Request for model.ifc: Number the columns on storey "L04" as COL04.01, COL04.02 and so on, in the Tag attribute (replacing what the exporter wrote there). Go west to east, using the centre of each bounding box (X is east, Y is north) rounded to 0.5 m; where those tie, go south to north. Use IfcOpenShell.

First a look at what the model holds.

```python
import ifcopenshell
import ifcopenshell.util.element
import ifcopenshell.util.placement

model = ifcopenshell.open("model.ifc")
print(model.schema)
storey = next(s for s in model.by_type("IfcBuildingStorey") if s.Name == "L04")
columns = [e for e in ifcopenshell.util.element.get_decomposition(storey) if e.is_a("IfcColumn")]
for e in sorted(columns, key=lambda e: e.id()):
    origin = ifcopenshell.util.placement.get_local_placement(e.ObjectPlacement)[:3, 3]
    print(e.id(), e.Tag, e.Name, origin.round(2) + 0.0, sep=" | ")
```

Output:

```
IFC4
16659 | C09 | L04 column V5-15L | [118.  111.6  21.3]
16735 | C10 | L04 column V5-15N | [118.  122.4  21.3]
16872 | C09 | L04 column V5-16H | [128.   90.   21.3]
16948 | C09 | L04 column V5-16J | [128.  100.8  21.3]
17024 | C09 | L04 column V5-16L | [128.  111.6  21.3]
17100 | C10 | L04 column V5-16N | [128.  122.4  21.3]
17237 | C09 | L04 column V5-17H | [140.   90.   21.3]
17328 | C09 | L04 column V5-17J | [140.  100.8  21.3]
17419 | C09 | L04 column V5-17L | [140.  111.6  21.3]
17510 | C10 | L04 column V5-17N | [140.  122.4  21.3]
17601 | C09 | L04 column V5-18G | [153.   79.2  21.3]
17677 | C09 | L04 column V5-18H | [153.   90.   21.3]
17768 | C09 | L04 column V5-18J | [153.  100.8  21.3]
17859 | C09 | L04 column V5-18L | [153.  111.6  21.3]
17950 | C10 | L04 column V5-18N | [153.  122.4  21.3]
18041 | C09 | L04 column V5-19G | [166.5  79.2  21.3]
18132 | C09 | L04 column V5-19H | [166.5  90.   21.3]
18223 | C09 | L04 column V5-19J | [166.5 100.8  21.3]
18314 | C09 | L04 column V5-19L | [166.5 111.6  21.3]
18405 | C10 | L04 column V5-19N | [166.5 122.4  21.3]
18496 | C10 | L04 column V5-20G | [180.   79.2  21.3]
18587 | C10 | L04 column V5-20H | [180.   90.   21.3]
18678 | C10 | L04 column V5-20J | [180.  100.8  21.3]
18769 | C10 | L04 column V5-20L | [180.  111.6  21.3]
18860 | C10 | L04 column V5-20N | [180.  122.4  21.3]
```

```python
import ifcopenshell
import ifcopenshell.geom
import ifcopenshell.util.element
import ifcopenshell.util.shape

model = ifcopenshell.open("model.ifc")
settings = ifcopenshell.geom.settings()
settings.set("use-world-coords", True)


def centre(element):
    shape = ifcopenshell.geom.create_shape(settings, element)
    return ifcopenshell.util.shape.get_bbox_centroid(shape.geometry)


storey = next(s for s in model.by_type("IfcBuildingStorey") if s.Name == "L04")
columns = [e for e in ifcopenshell.util.element.get_decomposition(storey) if e.is_a("IfcColumn")]

# Insertion points can sit at a corner or the storey origin, so sort by the geometry (in metres).
centres = {e: centre(e) for e in columns}
columns.sort(key=lambda e: (round(centres[e][0] / 0.5), centres[e][1]))

for i, e in enumerate(columns, start=1):
    number = f"COL04.{i:02d}"
    e.Tag = number
    print(e.id(), number)

model.write("model_edited.ifc")
```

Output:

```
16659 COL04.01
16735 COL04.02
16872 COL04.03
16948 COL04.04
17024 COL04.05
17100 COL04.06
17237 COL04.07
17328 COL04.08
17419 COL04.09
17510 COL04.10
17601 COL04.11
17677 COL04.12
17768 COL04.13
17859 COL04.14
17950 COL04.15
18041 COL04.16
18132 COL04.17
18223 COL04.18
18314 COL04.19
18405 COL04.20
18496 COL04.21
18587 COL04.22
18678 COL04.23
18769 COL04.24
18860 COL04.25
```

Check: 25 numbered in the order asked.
